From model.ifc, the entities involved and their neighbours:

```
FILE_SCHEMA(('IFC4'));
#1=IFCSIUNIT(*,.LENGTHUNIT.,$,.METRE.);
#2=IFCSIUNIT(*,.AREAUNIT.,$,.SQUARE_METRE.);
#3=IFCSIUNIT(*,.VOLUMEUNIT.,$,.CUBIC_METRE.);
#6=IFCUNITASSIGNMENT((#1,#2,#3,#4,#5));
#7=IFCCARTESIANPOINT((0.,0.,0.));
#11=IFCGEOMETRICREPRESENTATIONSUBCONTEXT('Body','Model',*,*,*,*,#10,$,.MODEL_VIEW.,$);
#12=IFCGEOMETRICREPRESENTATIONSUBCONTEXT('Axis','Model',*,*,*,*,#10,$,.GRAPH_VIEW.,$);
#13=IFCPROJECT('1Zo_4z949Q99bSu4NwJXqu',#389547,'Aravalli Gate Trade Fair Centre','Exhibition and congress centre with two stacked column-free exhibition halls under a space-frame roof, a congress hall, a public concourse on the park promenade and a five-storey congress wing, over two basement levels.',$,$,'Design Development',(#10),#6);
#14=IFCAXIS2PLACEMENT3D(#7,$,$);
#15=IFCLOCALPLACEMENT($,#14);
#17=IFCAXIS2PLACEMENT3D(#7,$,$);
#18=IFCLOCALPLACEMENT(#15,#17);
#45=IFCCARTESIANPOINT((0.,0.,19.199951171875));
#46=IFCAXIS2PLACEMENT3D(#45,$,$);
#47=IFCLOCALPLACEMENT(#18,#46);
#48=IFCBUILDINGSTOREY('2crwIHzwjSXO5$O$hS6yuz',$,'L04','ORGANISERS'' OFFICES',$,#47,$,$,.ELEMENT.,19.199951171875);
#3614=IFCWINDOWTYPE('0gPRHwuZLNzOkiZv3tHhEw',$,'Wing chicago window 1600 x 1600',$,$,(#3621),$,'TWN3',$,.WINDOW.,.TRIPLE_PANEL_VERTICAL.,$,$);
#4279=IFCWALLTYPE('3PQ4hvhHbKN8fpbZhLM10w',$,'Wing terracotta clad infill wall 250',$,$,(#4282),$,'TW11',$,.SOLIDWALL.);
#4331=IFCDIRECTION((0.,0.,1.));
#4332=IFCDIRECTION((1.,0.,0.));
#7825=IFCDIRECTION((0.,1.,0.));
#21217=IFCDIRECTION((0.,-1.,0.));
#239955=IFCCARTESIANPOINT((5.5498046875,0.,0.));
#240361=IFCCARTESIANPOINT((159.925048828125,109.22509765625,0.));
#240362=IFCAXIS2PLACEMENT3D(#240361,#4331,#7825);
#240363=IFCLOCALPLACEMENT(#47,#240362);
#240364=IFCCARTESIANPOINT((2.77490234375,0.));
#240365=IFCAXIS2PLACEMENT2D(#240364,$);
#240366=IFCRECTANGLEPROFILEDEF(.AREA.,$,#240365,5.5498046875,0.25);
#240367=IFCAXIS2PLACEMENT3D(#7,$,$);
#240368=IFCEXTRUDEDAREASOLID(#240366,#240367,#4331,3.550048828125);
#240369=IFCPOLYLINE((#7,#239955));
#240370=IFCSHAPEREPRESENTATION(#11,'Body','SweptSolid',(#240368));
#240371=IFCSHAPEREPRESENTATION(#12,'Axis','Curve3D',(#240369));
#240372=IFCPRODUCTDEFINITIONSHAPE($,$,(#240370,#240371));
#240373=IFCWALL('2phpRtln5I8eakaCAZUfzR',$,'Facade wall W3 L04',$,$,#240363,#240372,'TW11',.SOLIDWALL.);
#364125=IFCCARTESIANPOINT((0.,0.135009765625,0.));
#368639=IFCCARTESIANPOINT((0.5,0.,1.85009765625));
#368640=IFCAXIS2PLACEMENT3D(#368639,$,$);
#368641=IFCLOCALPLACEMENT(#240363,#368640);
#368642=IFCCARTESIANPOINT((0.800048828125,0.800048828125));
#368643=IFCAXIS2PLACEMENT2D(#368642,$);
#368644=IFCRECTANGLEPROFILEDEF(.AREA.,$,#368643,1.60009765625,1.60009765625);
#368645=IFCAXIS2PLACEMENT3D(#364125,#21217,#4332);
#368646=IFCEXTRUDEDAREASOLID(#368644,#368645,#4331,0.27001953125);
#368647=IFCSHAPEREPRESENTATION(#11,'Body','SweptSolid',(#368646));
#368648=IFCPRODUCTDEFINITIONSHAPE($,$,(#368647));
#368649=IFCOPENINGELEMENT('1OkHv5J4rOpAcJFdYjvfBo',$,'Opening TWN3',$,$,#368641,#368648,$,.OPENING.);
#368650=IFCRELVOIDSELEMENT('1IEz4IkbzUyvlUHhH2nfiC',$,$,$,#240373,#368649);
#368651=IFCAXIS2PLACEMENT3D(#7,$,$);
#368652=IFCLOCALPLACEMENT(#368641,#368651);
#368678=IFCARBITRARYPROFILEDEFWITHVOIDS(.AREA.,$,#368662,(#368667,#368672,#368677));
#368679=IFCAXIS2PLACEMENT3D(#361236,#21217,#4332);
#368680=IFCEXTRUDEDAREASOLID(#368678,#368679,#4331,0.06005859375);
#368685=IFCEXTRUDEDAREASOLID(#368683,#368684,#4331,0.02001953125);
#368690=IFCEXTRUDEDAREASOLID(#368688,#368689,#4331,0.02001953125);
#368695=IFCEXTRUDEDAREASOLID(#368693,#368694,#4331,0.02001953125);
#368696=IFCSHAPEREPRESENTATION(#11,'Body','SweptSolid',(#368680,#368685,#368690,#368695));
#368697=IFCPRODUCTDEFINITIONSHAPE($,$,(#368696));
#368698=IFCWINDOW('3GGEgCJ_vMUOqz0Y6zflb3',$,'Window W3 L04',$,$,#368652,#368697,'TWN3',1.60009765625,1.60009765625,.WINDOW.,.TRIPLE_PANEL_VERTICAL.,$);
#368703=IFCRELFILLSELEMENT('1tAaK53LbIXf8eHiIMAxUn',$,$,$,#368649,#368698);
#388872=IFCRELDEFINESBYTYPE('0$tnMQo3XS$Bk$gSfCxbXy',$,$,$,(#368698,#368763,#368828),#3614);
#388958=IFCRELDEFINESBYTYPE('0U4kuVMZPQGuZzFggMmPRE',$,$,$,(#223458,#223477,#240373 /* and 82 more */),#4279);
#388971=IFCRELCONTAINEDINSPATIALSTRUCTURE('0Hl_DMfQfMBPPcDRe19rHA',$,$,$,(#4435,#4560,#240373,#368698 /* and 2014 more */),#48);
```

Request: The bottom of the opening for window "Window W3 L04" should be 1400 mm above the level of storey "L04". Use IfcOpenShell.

```python
import numpy as np
import ifcopenshell
import ifcopenshell.api.geometry
import ifcopenshell.geom
import ifcopenshell.util.element
import ifcopenshell.util.placement
import ifcopenshell.util.shape
import ifcopenshell.util.unit

model = ifcopenshell.open("model.ifc")
unit_scale = ifcopenshell.util.unit.calculate_unit_scale(model)

window = model.by_id(368698)
opening = window.FillsVoids[0].RelatingOpeningElement
storey = ifcopenshell.util.element.get_container(window, ifc_class="IfcBuildingStorey")
level = ifcopenshell.util.placement.get_local_placement(storey.ObjectPlacement)[2, 3]

# The opening's origin need not be at the sill, so measure its lowest point.
shape = ifcopenshell.geom.create_shape(ifcopenshell.geom.settings(), opening)
bottom = ifcopenshell.util.shape.get_shape_bottom_elevation(shape, shape.geometry) / unit_scale
dz = level + 1.4 / unit_scale - bottom

shift = np.array([0.0, 0.0, dz])
# The window is placed relative to its opening, so it follows when the opening moves.
matrix = ifcopenshell.util.placement.get_local_placement(opening.ObjectPlacement)
matrix[:3, 3] += shift
ifcopenshell.api.geometry.edit_object_placement(
    model, product=opening, matrix=matrix, is_si=False, should_transform_children=True
)

print(f"moved by {dz * unit_scale:+.3f} m")

model.write("model-out.ifc")
```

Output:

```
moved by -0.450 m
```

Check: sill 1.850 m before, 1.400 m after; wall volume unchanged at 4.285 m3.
